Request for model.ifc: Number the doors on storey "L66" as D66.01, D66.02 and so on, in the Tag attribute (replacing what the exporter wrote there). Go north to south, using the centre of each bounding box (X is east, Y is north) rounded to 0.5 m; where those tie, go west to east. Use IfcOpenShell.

First a look at what the model holds.

```python
import ifcopenshell
import ifcopenshell.util.element
import ifcopenshell.util.placement

model = ifcopenshell.open("model.ifc")
print(model.schema)
storey = next(s for s in model.by_type("IfcBuildingStorey") if s.Name == "L66")
doors = [e for e in ifcopenshell.util.element.get_decomposition(storey) if e.is_a("IfcDoor")]
for e in sorted(doors, key=lambda e: e.id()):
    origin = ifcopenshell.util.placement.get_local_placement(e.ObjectPlacement)[:3, 3]
    print(e.id(), e.Tag, e.Name, origin.round(2) + 0.0, sep=" | ")
```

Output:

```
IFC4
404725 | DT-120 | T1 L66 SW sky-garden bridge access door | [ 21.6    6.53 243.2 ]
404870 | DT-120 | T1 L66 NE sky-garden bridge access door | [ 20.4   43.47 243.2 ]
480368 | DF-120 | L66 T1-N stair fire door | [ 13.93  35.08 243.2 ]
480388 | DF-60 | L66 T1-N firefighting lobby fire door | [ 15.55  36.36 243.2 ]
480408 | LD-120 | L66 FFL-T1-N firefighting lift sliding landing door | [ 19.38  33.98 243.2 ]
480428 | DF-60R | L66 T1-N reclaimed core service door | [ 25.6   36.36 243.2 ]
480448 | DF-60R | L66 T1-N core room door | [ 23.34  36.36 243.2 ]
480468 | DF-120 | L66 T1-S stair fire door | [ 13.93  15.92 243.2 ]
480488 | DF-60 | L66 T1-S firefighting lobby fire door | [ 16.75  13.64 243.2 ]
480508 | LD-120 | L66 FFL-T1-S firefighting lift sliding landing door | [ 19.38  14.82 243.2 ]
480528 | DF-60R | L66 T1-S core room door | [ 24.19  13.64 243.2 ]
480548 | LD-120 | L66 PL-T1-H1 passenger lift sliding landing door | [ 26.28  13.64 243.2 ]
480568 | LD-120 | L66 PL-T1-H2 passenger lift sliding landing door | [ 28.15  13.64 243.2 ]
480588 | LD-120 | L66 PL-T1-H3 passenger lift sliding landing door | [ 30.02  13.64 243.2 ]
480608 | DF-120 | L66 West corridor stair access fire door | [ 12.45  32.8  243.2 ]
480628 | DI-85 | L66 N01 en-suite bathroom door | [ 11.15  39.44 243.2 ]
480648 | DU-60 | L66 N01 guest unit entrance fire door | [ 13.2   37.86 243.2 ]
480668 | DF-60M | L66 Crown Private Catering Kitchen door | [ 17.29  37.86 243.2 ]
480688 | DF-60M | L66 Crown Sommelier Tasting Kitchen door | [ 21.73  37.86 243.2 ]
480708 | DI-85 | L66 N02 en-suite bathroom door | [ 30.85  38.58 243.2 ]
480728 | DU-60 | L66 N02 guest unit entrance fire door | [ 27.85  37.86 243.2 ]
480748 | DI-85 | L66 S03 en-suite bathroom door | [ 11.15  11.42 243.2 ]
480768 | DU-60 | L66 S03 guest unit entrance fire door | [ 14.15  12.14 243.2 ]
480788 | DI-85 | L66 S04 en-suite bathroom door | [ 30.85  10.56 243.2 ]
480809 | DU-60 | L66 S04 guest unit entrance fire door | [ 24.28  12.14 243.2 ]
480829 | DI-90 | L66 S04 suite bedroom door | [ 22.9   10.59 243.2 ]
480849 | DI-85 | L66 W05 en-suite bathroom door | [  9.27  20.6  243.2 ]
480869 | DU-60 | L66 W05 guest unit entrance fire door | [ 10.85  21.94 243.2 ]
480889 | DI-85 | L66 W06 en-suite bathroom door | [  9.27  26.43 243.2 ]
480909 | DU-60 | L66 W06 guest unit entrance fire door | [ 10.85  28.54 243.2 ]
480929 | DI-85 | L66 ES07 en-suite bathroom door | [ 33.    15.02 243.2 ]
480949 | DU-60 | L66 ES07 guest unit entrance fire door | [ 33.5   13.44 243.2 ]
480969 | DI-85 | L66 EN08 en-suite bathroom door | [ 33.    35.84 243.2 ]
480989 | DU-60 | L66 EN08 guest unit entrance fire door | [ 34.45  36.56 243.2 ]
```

```python
import ifcopenshell
import ifcopenshell.geom
import ifcopenshell.util.element
import ifcopenshell.util.shape

model = ifcopenshell.open("model.ifc")
settings = ifcopenshell.geom.settings()
settings.set("use-world-coords", True)


def centre(element):
    shape = ifcopenshell.geom.create_shape(settings, element)
    return ifcopenshell.util.shape.get_bbox_centroid(shape.geometry)


storey = next(s for s in model.by_type("IfcBuildingStorey") if s.Name == "L66")
doors = [e for e in ifcopenshell.util.element.get_decomposition(storey) if e.is_a("IfcDoor")]

# Insertion points can sit at a corner or the storey origin, so sort by the geometry (in metres).
centres = {e: centre(e) for e in doors}
doors.sort(key=lambda e: (-round(centres[e][1] / 0.5), centres[e][0]))

for i, e in enumerate(doors, start=1):
    number = f"D66.{i:02d}"
    e.Tag = number
    print(e.id(), number)

model.write("model_rev.ifc")
```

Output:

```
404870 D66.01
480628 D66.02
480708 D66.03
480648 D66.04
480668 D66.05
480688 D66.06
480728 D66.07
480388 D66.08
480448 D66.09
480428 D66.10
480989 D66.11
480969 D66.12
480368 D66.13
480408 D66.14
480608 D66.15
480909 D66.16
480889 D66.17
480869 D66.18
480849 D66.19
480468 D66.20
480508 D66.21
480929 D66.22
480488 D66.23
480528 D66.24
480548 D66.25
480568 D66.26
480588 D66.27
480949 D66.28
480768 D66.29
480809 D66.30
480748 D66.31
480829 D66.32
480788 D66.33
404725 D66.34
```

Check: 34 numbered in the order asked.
